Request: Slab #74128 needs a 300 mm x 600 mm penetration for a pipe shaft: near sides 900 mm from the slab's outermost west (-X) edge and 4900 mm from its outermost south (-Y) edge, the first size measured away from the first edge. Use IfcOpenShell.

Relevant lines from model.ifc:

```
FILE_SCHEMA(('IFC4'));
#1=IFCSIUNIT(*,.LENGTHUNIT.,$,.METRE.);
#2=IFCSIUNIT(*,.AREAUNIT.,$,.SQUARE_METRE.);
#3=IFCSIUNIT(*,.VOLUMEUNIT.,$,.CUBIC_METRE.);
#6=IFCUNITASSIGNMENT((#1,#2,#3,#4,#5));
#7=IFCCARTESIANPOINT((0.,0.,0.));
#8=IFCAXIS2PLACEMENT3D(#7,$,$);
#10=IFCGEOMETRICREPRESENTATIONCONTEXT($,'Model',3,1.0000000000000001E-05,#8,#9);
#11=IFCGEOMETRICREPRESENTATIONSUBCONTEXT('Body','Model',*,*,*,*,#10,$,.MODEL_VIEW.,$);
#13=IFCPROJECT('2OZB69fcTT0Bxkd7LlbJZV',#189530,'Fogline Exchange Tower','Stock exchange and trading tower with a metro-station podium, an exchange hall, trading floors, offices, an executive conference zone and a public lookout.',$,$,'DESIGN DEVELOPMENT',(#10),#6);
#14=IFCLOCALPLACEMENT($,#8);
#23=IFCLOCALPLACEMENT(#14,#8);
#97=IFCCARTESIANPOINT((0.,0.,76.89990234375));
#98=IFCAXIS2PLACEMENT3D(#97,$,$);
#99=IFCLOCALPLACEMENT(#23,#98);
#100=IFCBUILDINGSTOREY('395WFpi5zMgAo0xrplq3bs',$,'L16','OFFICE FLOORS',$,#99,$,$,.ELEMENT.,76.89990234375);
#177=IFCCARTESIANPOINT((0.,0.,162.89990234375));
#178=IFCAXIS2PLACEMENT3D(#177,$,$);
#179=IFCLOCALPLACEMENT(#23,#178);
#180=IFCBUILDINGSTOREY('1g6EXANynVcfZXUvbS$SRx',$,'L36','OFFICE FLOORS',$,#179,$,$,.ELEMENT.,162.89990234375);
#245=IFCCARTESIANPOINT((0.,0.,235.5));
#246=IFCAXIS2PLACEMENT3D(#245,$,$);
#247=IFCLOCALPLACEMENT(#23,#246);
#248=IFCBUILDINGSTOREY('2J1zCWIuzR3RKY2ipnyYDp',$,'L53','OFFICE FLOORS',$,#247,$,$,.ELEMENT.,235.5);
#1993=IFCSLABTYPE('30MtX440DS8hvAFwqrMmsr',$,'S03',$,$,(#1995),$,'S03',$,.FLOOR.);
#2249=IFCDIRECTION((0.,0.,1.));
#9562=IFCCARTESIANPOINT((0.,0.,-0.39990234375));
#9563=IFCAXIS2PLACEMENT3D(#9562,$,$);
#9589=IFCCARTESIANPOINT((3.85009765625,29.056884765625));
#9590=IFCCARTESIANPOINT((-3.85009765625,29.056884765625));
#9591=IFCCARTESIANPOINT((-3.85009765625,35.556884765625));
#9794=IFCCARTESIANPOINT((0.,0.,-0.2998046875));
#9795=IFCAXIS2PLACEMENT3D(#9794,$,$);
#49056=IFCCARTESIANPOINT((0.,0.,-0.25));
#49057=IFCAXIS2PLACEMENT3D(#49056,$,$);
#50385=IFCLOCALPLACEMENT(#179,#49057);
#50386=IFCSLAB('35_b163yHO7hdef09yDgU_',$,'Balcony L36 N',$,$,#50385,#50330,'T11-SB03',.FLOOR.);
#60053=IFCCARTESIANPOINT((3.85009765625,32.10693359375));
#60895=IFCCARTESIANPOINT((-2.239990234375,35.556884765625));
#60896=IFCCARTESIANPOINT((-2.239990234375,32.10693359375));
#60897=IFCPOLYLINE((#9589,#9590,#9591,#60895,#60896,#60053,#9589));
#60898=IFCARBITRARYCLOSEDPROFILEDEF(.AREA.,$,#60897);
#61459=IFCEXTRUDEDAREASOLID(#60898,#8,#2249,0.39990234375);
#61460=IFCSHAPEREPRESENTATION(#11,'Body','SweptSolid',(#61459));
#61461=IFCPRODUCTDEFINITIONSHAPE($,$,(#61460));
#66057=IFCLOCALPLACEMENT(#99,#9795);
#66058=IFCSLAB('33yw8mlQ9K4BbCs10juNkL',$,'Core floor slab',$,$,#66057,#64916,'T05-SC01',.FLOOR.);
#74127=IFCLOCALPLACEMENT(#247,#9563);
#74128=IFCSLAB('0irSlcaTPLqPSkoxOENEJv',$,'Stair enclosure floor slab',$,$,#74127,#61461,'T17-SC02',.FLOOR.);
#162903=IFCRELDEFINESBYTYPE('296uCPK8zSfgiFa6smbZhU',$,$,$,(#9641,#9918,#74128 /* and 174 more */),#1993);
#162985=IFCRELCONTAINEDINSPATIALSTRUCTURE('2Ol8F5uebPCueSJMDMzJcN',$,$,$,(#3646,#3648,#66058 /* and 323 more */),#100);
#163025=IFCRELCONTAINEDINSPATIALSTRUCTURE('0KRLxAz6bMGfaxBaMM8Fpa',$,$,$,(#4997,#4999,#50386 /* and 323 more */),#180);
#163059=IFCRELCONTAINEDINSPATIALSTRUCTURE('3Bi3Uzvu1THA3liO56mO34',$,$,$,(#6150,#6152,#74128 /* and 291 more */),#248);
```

```python
import numpy as np
import ifcopenshell
import ifcopenshell.api.feature
import ifcopenshell.api.geometry
import ifcopenshell.api.root
import ifcopenshell.geom
import ifcopenshell.util.placement
import ifcopenshell.util.representation
import ifcopenshell.util.shape
import ifcopenshell.util.unit

model = ifcopenshell.open("model.ifc")
unit_scale = ifcopenshell.util.unit.calculate_unit_scale(model)
settings = ifcopenshell.geom.settings()


def volume(element):
    """Net volume in cubic metres, openings subtracted."""
    shape = ifcopenshell.geom.create_shape(settings, element)
    return ifcopenshell.util.shape.get_volume(shape.geometry)


slab = model.by_id(74128)
before = volume(slab)

# Extent in the slab's own axes, in metres. The edges named are its -X and -Y sides.
slab_shape = ifcopenshell.geom.create_shape(settings, slab)
vertices = ifcopenshell.util.shape.get_vertices(slab_shape.geometry)
x_min, y_min, bottom = vertices.min(axis=0)
top = vertices[:, 2].max()

opening = ifcopenshell.api.root.create_entity(model, ifc_class="IfcOpeningElement", name="Pipe shaft opening", predefined_type="OPENING")
context = ifcopenshell.util.representation.get_context(model, "Model", "Body", "MODEL_VIEW")
width, depth = 0.3, 0.6
outline = [(0.0, 0.0), (width, 0.0), (width, depth), (0.0, depth), (0.0, 0.0)]
# Overshoot both faces by 50 mm so the cut is clean.
shape = ifcopenshell.api.geometry.add_slab_representation(
    model, context=context, depth=top - bottom + 0.1, polyline=outline
)
ifcopenshell.api.geometry.assign_representation(model, product=opening, representation=shape)

matrix = ifcopenshell.util.placement.get_local_placement(slab.ObjectPlacement)
matrix[:, 3] = matrix @ np.append(np.array([x_min + 0.9, y_min + 4.9, bottom - 0.05]) / unit_scale, 1.0)
ifcopenshell.api.geometry.edit_object_placement(model, product=opening, matrix=matrix, is_si=False)
ifcopenshell.api.feature.add_feature(model, feature=opening, element=slab)

after = volume(slab)

print(f"slab volume {before:.3f} -> {after:.3f} m3")

model.write("model_edited.ifc")
```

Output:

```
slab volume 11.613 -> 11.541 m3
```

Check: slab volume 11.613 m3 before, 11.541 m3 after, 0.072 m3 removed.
